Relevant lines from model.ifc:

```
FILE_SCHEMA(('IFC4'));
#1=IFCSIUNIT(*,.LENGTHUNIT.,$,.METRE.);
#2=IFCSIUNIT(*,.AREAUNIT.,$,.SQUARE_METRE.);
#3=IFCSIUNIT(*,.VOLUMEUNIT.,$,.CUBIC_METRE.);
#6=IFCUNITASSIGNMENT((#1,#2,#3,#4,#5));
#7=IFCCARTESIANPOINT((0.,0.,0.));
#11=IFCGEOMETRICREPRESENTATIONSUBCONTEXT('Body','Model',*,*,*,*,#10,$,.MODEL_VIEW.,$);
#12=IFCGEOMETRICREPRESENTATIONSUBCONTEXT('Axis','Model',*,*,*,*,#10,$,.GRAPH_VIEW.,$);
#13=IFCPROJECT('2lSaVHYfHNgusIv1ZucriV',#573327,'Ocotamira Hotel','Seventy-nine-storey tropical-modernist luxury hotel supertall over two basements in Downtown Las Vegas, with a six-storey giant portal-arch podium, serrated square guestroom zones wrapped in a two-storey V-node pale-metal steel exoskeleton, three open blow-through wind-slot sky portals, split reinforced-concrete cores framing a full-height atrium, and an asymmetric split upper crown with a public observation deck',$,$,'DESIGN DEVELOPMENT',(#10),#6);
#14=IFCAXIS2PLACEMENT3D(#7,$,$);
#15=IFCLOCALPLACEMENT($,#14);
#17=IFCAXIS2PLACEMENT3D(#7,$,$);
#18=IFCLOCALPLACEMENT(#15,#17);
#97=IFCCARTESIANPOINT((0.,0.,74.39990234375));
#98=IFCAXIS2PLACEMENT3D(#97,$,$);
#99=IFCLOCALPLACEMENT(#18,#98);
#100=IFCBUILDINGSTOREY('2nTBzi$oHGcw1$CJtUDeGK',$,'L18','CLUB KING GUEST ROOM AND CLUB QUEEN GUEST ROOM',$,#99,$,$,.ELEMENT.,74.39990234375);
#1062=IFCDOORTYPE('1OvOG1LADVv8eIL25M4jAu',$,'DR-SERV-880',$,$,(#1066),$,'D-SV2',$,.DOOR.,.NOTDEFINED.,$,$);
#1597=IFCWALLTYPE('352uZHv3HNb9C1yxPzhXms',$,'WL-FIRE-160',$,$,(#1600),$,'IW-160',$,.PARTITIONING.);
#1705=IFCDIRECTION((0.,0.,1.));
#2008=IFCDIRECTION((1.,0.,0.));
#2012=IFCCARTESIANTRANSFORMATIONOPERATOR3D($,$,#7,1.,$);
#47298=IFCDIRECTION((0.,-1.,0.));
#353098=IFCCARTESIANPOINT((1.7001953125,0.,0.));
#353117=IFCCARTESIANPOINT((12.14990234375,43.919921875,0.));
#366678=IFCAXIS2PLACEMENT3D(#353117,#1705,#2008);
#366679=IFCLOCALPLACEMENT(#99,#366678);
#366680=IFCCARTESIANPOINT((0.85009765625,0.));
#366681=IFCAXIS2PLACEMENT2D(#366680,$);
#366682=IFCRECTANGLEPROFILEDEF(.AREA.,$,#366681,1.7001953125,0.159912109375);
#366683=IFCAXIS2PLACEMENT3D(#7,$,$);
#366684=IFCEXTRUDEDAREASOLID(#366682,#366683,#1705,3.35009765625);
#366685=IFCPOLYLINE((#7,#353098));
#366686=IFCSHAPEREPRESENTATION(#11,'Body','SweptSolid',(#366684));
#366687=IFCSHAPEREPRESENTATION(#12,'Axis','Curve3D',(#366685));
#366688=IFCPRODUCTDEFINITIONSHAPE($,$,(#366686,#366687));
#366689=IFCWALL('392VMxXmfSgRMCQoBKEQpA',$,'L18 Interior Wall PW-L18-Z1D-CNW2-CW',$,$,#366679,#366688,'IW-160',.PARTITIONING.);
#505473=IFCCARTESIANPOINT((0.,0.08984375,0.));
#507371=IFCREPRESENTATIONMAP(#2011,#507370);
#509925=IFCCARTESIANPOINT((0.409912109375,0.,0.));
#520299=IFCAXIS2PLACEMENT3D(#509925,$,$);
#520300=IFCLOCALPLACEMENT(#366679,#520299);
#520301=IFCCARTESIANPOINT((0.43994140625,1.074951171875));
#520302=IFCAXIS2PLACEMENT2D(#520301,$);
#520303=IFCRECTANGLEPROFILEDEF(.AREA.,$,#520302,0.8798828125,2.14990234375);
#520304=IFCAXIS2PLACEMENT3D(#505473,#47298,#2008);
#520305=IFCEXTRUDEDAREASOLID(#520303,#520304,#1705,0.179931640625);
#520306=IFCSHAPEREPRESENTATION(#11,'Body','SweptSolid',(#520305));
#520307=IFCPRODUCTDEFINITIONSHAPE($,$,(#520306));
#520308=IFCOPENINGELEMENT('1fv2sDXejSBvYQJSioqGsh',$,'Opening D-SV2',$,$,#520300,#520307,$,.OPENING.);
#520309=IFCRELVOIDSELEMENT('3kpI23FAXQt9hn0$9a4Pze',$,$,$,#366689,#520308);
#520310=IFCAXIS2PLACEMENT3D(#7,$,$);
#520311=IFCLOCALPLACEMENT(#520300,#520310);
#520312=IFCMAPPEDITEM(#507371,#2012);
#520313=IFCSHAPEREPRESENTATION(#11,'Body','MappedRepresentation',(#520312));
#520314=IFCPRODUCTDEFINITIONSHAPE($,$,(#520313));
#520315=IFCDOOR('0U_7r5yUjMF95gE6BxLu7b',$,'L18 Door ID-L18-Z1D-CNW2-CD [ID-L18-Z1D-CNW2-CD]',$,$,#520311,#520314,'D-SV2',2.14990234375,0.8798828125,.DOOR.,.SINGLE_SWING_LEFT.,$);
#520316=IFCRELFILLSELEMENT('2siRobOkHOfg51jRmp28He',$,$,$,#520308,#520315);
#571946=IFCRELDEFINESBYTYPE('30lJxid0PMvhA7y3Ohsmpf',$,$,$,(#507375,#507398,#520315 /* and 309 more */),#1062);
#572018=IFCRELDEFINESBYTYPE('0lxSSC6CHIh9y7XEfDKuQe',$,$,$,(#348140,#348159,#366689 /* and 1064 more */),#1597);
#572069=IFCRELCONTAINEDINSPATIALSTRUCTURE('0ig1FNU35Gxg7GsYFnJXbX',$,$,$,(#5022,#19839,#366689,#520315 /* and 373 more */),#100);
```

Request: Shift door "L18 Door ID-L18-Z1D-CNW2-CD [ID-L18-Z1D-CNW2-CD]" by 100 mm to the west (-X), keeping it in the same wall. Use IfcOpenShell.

```python
import ifcopenshell
import ifcopenshell.api.geometry
import ifcopenshell.util.placement
import ifcopenshell.util.unit

model = ifcopenshell.open("model.ifc")
unit_scale = ifcopenshell.util.unit.calculate_unit_scale(model)

door = model.by_guid("0U_7r5yUjMF95gE6BxLu7b")
opening = door.FillsVoids[0].RelatingOpeningElement
wall = opening.VoidsElements[0].RelatingBuildingElement

wall_matrix = ifcopenshell.util.placement.get_local_placement(wall.ObjectPlacement)
shift = wall_matrix[:3, 0] * -0.1 / unit_scale
before = ifcopenshell.util.placement.get_local_placement(door.ObjectPlacement)[:3, 3].copy()

# The door is placed relative to its opening, so it follows when the opening moves.
matrix = ifcopenshell.util.placement.get_local_placement(opening.ObjectPlacement)
matrix[:3, 3] += shift
ifcopenshell.api.geometry.edit_object_placement(
    model, product=opening, matrix=matrix, is_si=False, should_transform_children=True
)

after = ifcopenshell.util.placement.get_local_placement(door.ObjectPlacement)[:3, 3]
print("door moved by", (after - before).round(3) + 0.0)

model.write("model_edited.ifc")
```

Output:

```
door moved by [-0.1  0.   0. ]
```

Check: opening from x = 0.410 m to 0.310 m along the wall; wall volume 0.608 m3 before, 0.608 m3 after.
